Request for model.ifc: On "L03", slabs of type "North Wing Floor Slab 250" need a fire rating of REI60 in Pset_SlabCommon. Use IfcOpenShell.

First a look at what the model holds.

```python
import ifcopenshell
import ifcopenshell.util.element

model = ifcopenshell.open("model.ifc")
print(model.schema)
storey = next(s for s in model.by_type("IfcBuildingStorey") if s.Name == "L03")
slabs = [e for e in ifcopenshell.util.element.get_decomposition(storey) if e.is_a("IfcSlab")]
seen = {}
for e in slabs:
    element_type = ifcopenshell.util.element.get_type(e)
    key = (element_type.Name if element_type != e and element_type else None, ifcopenshell.util.element.get_pset(e, "Pset_SlabCommon", "FireRating"))
    seen[key] = seen.get(key, 0) + 1
for (name, value), count in sorted(seen.items(), key=str):
    print(count, "x", name, "|", value)
```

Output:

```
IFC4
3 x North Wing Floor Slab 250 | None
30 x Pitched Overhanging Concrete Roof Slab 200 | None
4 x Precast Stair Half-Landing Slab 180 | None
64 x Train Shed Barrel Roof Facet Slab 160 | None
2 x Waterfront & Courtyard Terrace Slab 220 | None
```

```python
import ifcopenshell
import ifcopenshell.api.pset
import ifcopenshell.util.element

model = ifcopenshell.open("model.ifc")

storey = next(s for s in model.by_type("IfcBuildingStorey") if s.Name == "L03")
slabs = [e for e in ifcopenshell.util.element.get_decomposition(storey) if e.is_a("IfcSlab")]

count = 0
for e in slabs:
    element_type = ifcopenshell.util.element.get_type(e)
    if element_type in (None, e) or element_type.Name != "North Wing Floor Slab 250":
        continue
    # add_pset returns the element's existing set when there is one.
    pset = ifcopenshell.api.pset.add_pset(model, product=e, name="Pset_SlabCommon")
    ifcopenshell.api.pset.edit_pset(model, pset=pset, properties={"FireRating": "REI60"})
    count += 1

print(count, "slabs updated")

model.write("model_rev.ifc")
```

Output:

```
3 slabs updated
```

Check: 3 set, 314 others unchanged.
